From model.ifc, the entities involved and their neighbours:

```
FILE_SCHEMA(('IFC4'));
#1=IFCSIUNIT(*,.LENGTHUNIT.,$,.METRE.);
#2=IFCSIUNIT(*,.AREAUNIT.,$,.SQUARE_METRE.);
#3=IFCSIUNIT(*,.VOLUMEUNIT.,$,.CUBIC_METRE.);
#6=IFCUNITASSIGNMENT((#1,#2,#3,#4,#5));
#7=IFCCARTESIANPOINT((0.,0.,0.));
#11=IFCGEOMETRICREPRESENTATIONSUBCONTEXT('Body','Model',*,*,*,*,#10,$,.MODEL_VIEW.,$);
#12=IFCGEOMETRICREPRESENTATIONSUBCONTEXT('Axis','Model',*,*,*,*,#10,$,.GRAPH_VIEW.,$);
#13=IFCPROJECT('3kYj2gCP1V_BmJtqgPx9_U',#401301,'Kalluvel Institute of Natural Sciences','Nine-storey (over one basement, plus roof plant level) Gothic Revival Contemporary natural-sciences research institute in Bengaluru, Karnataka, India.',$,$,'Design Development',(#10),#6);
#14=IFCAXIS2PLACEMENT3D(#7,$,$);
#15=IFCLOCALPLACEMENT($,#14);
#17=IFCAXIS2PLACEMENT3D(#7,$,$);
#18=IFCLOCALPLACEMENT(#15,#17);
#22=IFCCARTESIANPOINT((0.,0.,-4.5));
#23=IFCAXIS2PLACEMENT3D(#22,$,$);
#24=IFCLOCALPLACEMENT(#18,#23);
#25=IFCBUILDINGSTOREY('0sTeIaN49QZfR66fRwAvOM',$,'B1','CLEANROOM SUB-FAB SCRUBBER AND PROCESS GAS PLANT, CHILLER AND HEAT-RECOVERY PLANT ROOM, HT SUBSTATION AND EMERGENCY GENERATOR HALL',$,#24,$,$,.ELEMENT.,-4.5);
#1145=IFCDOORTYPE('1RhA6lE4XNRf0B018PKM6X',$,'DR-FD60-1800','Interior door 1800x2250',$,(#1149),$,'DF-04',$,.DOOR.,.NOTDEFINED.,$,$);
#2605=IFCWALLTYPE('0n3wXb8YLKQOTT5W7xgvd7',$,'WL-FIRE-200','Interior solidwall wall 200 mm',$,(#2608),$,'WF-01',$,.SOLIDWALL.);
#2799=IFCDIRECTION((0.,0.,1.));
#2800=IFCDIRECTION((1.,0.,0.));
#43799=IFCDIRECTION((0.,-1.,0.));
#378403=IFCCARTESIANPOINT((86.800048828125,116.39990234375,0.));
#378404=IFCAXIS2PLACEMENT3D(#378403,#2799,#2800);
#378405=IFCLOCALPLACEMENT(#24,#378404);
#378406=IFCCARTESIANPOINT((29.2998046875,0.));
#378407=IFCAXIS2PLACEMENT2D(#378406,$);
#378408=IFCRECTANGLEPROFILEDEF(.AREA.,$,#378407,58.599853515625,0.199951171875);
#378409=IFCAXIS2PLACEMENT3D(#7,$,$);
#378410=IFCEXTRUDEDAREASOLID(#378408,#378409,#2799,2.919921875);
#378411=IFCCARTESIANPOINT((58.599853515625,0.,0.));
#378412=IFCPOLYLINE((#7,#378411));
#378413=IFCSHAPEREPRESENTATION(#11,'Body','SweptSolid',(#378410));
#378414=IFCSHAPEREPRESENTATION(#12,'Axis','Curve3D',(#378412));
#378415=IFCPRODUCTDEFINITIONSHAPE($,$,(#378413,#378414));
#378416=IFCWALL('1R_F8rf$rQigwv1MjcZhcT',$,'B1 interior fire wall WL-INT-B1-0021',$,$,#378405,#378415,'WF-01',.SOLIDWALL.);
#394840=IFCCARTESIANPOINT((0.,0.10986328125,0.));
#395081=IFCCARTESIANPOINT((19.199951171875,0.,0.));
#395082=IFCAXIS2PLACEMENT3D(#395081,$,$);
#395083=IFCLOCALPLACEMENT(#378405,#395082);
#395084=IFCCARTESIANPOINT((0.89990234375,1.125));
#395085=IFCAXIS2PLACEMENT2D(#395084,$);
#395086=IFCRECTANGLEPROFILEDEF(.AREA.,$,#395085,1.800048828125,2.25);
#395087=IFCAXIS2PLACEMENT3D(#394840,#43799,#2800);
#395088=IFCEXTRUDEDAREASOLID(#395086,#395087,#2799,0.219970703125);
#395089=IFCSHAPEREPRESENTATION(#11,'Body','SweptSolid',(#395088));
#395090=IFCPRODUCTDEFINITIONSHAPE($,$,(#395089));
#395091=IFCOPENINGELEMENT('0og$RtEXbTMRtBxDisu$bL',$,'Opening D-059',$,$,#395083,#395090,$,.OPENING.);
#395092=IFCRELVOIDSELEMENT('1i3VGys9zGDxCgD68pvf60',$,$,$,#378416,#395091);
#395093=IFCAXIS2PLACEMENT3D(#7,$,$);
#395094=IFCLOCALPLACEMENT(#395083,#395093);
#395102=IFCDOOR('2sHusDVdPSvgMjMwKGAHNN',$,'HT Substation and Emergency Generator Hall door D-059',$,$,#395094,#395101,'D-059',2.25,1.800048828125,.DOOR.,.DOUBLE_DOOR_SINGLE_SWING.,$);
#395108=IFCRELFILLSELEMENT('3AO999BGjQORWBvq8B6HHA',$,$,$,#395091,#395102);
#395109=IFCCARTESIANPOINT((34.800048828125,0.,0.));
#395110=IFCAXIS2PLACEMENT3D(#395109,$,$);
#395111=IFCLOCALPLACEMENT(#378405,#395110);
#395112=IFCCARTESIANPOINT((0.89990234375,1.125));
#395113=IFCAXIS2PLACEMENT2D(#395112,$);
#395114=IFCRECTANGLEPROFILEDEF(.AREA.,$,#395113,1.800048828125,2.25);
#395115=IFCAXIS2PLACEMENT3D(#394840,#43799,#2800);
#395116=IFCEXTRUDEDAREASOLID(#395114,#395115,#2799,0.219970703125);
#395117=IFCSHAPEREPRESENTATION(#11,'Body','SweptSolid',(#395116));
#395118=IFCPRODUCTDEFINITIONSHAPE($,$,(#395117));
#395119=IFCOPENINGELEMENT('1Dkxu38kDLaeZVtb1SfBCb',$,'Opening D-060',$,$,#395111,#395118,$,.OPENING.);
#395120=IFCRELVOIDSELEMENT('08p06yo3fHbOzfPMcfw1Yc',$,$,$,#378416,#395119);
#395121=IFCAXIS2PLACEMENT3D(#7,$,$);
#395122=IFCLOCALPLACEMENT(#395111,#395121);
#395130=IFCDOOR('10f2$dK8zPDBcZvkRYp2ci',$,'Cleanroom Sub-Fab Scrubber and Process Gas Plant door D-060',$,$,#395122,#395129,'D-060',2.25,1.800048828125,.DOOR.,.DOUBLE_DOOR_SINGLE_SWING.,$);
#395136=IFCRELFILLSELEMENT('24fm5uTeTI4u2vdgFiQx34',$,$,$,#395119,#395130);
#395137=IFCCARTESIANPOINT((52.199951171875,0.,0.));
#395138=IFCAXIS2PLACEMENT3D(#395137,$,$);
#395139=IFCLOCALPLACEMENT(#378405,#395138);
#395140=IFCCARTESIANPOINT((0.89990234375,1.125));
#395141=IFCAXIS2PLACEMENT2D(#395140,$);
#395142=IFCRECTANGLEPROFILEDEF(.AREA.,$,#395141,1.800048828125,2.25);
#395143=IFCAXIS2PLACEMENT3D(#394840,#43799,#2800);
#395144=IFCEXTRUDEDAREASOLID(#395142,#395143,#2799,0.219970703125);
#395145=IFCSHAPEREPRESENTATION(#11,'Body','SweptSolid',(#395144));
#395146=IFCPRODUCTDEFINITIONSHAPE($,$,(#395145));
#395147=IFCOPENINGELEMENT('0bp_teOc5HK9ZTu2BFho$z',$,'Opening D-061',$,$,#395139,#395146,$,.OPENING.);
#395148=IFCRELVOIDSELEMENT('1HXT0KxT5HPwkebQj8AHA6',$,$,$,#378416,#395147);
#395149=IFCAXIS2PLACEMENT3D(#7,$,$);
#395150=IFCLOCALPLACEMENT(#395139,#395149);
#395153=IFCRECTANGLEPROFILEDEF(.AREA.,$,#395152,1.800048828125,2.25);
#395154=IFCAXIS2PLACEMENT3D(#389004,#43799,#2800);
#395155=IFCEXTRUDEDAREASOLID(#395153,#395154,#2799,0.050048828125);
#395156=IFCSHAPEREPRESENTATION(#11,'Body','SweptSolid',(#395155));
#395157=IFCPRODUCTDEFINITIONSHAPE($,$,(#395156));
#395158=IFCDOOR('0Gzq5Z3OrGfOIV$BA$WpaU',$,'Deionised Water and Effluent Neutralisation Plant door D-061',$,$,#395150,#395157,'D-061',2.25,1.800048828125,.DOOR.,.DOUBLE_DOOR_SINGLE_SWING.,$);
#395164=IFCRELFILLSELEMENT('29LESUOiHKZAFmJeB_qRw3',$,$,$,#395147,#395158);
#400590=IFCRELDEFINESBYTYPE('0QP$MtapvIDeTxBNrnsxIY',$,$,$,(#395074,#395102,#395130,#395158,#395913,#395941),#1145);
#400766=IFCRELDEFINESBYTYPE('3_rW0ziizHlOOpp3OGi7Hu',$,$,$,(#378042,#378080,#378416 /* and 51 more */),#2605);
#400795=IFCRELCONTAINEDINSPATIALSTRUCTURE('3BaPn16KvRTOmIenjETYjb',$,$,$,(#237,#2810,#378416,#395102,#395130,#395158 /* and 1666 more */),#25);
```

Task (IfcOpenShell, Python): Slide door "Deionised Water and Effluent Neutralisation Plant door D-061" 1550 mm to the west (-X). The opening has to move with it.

```python
import ifcopenshell
import ifcopenshell.api.geometry
import ifcopenshell.util.placement
import ifcopenshell.util.unit

model = ifcopenshell.open("model.ifc")
unit_scale = ifcopenshell.util.unit.calculate_unit_scale(model)

door = model.by_guid("0Gzq5Z3OrGfOIV$BA$WpaU")
opening = door.FillsVoids[0].RelatingOpeningElement
wall = opening.VoidsElements[0].RelatingBuildingElement

wall_matrix = ifcopenshell.util.placement.get_local_placement(wall.ObjectPlacement)
shift = wall_matrix[:3, 0] * -1.55 / unit_scale
before = ifcopenshell.util.placement.get_local_placement(door.ObjectPlacement)[:3, 3].copy()

# The door is placed relative to its opening, so it follows when the opening moves.
matrix = ifcopenshell.util.placement.get_local_placement(opening.ObjectPlacement)
matrix[:3, 3] += shift
ifcopenshell.api.geometry.edit_object_placement(
    model, product=opening, matrix=matrix, is_si=False, should_transform_children=True
)

after = ifcopenshell.util.placement.get_local_placement(door.ObjectPlacement)[:3, 3]
print("door moved by", (after - before).round(3) + 0.0)

model.write("model_rev.ifc")
```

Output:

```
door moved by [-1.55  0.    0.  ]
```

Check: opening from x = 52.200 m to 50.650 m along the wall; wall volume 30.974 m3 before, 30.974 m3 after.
